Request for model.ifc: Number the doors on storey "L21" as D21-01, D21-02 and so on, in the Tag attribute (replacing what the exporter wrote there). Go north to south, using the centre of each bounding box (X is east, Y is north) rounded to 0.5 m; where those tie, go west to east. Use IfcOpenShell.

First a look at what the model holds.

```python
import ifcopenshell
import ifcopenshell.util.element
import ifcopenshell.util.placement

model = ifcopenshell.open("model.ifc")
print(model.schema)
storey = next(s for s in model.by_type("IfcBuildingStorey") if s.Name == "L21")
doors = [e for e in ifcopenshell.util.element.get_decomposition(storey) if e.is_a("IfcDoor")]
for e in sorted(doors, key=lambda e: e.id()):
    origin = ifcopenshell.util.placement.get_local_placement(e.ObjectPlacement)[:3, 3]
    print(e.id(), e.Tag, e.Name, origin.round(2) + 0.0, sep=" | ")
```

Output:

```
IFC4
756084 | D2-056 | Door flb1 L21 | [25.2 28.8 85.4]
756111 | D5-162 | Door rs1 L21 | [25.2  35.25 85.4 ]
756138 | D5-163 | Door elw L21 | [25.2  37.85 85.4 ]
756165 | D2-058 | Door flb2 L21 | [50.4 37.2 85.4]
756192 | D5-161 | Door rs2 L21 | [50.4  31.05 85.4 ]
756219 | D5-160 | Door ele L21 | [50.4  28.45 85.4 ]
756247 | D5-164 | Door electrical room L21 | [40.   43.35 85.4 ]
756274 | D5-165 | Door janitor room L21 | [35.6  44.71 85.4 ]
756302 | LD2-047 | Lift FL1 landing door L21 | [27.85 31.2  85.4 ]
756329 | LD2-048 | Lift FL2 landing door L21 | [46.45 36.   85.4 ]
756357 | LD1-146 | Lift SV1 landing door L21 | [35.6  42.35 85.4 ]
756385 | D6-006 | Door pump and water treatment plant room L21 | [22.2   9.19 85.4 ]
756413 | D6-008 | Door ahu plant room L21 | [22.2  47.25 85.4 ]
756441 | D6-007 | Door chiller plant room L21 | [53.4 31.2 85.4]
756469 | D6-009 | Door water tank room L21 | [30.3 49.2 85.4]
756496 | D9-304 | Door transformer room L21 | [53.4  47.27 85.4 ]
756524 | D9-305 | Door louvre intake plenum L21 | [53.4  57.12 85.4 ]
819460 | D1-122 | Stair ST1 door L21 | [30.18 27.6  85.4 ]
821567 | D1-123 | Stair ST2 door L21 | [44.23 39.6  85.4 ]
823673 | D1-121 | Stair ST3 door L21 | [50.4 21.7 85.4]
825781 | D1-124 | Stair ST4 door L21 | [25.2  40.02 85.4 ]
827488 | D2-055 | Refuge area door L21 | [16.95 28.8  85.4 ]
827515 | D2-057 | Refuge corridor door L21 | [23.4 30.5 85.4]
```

```python
import ifcopenshell
import ifcopenshell.geom
import ifcopenshell.util.element
import ifcopenshell.util.shape

model = ifcopenshell.open("model.ifc")
settings = ifcopenshell.geom.settings()
settings.set("use-world-coords", True)


def centre(element):
    shape = ifcopenshell.geom.create_shape(settings, element)
    return ifcopenshell.util.shape.get_bbox_centroid(shape.geometry)


storey = next(s for s in model.by_type("IfcBuildingStorey") if s.Name == "L21")
doors = [e for e in ifcopenshell.util.element.get_decomposition(storey) if e.is_a("IfcDoor")]

# Insertion points can sit at a corner or the storey origin, so sort by the geometry (in metres).
centres = {e: centre(e) for e in doors}
doors.sort(key=lambda e: (-round(centres[e][1] / 0.5), centres[e][0]))

for i, e in enumerate(doors, start=1):
    number = f"D21-{i:02d}"
    e.Tag = number
    print(e.id(), number)

model.write("model_edited.ifc")
```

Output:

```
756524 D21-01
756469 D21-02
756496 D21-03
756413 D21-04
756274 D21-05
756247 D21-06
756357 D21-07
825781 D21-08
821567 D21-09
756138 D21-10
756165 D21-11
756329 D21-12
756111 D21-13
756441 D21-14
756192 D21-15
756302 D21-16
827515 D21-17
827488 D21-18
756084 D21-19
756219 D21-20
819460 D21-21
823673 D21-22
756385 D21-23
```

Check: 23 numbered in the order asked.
